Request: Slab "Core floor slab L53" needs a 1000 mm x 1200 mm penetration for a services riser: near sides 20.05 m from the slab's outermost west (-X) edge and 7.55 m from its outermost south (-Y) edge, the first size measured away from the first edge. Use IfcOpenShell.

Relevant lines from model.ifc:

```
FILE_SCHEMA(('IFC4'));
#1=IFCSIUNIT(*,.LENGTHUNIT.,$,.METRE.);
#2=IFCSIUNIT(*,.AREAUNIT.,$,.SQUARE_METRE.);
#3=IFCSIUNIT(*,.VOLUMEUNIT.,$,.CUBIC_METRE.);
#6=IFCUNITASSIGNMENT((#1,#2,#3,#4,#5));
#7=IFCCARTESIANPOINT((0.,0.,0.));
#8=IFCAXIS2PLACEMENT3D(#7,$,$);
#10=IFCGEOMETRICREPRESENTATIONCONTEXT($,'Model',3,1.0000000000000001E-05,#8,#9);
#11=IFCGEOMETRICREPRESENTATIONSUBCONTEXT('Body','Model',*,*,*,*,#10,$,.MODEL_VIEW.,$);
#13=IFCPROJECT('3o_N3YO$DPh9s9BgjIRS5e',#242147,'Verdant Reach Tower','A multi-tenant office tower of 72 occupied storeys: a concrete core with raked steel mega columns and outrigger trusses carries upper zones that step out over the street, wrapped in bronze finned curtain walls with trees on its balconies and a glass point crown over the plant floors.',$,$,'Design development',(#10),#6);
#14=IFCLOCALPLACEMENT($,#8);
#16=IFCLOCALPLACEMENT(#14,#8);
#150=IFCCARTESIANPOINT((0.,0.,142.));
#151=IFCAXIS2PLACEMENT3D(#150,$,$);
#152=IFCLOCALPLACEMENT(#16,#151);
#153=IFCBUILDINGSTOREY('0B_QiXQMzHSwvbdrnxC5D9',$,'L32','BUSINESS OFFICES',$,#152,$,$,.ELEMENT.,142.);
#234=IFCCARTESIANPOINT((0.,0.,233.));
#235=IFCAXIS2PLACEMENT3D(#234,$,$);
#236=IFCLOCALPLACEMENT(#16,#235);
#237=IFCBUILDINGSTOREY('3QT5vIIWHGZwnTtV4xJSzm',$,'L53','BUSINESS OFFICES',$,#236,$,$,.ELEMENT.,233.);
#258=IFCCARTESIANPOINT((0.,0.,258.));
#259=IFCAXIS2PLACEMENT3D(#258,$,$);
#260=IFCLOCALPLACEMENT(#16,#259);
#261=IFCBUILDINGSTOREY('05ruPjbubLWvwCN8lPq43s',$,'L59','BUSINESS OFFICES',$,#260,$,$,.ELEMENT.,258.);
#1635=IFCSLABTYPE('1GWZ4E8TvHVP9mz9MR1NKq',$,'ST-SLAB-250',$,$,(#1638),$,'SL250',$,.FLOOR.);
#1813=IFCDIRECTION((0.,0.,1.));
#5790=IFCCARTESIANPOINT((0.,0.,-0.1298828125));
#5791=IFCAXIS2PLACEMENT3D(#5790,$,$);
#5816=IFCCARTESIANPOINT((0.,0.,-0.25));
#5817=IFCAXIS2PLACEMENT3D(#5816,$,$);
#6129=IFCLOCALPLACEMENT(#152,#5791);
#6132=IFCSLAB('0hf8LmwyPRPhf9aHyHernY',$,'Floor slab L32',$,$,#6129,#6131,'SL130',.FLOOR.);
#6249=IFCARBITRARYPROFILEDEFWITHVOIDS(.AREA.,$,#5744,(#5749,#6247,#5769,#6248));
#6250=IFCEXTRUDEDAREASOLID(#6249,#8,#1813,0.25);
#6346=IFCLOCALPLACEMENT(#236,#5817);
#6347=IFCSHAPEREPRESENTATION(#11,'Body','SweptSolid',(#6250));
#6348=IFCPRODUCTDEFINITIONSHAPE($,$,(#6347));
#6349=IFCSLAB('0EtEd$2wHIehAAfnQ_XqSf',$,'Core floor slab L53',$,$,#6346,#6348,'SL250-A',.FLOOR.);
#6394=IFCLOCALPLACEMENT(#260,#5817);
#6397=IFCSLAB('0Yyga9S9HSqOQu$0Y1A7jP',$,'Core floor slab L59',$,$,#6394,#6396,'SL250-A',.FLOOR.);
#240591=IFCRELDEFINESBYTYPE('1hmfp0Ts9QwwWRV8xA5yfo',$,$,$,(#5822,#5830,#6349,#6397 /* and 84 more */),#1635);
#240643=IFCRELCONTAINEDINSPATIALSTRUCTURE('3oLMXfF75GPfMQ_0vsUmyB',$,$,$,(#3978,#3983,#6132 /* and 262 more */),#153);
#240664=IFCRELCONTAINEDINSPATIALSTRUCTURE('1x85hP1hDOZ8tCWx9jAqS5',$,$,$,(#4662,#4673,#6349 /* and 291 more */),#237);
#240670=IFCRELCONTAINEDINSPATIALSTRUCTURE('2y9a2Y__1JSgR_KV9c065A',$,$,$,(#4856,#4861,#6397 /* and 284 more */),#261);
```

```python
import numpy as np
import ifcopenshell
import ifcopenshell.api.feature
import ifcopenshell.api.geometry
import ifcopenshell.api.root
import ifcopenshell.geom
import ifcopenshell.util.placement
import ifcopenshell.util.representation
import ifcopenshell.util.shape
import ifcopenshell.util.unit

model = ifcopenshell.open("model.ifc")
unit_scale = ifcopenshell.util.unit.calculate_unit_scale(model)
settings = ifcopenshell.geom.settings()


def volume(element):
    """Net volume in cubic metres, openings subtracted."""
    shape = ifcopenshell.geom.create_shape(settings, element)
    return ifcopenshell.util.shape.get_volume(shape.geometry)


slab = model.by_guid("0EtEd$2wHIehAAfnQ_XqSf")
before = volume(slab)

# Extent in the slab's own axes, in metres. The edges named are its -X and -Y sides.
slab_shape = ifcopenshell.geom.create_shape(settings, slab)
vertices = ifcopenshell.util.shape.get_vertices(slab_shape.geometry)
x_min, y_min, bottom = vertices.min(axis=0)
top = vertices[:, 2].max()

opening = ifcopenshell.api.root.create_entity(model, ifc_class="IfcOpeningElement", name="Services riser opening", predefined_type="OPENING")
context = ifcopenshell.util.representation.get_context(model, "Model", "Body", "MODEL_VIEW")
width, depth = 1, 1.2
outline = [(0.0, 0.0), (width, 0.0), (width, depth), (0.0, depth), (0.0, 0.0)]
# Overshoot both faces by 50 mm so the cut is clean.
shape = ifcopenshell.api.geometry.add_slab_representation(
    model, context=context, depth=top - bottom + 0.1, polyline=outline
)
ifcopenshell.api.geometry.assign_representation(model, product=opening, representation=shape)

matrix = ifcopenshell.util.placement.get_local_placement(slab.ObjectPlacement)
matrix[:, 3] = matrix @ np.append(np.array([x_min + 20.05, y_min + 7.55, bottom - 0.05]) / unit_scale, 1.0)
ifcopenshell.api.geometry.edit_object_placement(model, product=opening, matrix=matrix, is_si=False)
ifcopenshell.api.feature.add_feature(model, feature=opening, element=slab)

after = volume(slab)

print(f"slab volume {before:.3f} -> {after:.3f} m3")

model.write("model_rev.ifc")
```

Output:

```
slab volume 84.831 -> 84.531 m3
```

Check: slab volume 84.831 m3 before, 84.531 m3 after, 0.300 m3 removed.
